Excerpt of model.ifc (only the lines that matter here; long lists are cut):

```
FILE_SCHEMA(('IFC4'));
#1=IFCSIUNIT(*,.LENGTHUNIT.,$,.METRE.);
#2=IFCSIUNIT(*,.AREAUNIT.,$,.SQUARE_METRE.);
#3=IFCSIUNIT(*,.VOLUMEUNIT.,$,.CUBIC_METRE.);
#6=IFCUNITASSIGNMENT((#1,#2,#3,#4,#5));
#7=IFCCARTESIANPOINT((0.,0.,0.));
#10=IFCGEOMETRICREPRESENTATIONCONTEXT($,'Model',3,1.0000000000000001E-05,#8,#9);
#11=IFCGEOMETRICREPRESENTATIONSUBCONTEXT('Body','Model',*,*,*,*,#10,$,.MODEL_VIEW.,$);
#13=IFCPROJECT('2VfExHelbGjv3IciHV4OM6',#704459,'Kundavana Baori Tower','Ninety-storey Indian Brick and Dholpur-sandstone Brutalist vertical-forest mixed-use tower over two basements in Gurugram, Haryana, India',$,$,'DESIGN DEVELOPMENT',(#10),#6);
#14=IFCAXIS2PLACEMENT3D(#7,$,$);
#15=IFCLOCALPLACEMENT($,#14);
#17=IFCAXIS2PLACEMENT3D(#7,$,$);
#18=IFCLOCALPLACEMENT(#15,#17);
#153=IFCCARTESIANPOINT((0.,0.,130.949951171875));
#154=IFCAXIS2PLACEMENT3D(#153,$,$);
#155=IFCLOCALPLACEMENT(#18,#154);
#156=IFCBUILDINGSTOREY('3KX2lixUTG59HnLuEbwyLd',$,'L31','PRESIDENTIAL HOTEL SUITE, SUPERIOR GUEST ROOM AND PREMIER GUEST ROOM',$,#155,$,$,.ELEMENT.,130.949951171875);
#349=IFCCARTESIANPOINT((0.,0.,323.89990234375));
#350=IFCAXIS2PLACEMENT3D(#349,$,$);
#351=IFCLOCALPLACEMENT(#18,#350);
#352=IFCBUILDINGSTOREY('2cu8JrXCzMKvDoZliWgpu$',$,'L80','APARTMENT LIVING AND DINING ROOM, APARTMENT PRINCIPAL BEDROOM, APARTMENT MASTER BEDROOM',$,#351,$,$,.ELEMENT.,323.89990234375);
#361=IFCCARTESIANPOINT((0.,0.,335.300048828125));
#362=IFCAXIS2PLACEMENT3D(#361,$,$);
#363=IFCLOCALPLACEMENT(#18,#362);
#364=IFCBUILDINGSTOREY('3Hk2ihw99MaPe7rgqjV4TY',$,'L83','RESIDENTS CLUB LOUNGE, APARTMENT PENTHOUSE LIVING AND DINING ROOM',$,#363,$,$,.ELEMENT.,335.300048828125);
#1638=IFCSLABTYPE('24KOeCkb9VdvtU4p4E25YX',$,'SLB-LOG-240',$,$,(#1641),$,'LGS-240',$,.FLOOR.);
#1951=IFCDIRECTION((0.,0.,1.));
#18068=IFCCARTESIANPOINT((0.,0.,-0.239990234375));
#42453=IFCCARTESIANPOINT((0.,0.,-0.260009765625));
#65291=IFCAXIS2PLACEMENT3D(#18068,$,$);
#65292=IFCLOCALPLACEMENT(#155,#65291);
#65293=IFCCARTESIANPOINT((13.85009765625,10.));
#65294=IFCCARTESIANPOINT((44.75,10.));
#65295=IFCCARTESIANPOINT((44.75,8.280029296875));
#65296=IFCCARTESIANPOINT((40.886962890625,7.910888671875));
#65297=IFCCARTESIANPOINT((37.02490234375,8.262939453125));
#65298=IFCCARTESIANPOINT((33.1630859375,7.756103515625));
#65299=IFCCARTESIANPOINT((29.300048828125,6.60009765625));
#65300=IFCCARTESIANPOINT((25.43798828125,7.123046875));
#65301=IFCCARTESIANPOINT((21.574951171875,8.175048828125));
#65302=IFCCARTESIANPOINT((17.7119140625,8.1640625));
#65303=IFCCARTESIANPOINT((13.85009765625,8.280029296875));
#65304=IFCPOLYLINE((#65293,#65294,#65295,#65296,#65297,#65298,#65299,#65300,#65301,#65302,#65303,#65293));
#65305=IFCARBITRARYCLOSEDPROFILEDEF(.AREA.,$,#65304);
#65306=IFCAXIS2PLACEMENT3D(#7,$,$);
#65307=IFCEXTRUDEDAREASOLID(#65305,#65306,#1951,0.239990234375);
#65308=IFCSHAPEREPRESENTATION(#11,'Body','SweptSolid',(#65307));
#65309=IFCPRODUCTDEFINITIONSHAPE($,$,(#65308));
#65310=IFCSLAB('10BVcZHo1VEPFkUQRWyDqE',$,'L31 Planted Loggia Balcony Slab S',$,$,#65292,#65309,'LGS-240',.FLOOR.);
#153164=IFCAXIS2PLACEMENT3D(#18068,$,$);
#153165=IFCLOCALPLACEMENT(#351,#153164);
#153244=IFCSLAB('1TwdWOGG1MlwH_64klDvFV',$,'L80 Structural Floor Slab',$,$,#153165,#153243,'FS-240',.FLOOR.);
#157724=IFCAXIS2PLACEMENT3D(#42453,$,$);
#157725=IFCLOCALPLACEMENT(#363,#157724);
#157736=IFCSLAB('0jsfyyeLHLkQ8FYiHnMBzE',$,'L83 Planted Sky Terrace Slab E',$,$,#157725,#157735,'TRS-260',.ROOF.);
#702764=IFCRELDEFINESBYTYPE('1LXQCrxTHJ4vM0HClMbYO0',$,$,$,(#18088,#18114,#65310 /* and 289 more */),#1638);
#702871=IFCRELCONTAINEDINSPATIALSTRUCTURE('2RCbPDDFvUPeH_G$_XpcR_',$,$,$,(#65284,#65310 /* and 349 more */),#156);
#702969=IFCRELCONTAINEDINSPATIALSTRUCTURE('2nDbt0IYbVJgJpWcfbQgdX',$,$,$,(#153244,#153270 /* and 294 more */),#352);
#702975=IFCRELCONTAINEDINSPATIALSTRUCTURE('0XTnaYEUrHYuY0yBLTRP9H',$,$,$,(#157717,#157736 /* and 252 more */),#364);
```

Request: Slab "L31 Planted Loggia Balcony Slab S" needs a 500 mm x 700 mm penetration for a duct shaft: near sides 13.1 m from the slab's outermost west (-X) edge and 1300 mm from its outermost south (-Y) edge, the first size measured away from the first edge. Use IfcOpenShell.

```python
import numpy as np
import ifcopenshell
import ifcopenshell.api.feature
import ifcopenshell.api.geometry
import ifcopenshell.api.root
import ifcopenshell.geom
import ifcopenshell.util.placement
import ifcopenshell.util.representation
import ifcopenshell.util.shape
import ifcopenshell.util.unit

model = ifcopenshell.open("model.ifc")
unit_scale = ifcopenshell.util.unit.calculate_unit_scale(model)
settings = ifcopenshell.geom.settings()


def volume(element):
    """Net volume in cubic metres, openings subtracted."""
    shape = ifcopenshell.geom.create_shape(settings, element)
    return ifcopenshell.util.shape.get_volume(shape.geometry)


slab = model.by_id(65310)
before = volume(slab)

# Extent in the slab's own axes, in metres. The edges named are its -X and -Y sides.
slab_shape = ifcopenshell.geom.create_shape(settings, slab)
vertices = ifcopenshell.util.shape.get_vertices(slab_shape.geometry)
x_min, y_min, bottom = vertices.min(axis=0)
top = vertices[:, 2].max()

opening = ifcopenshell.api.root.create_entity(model, ifc_class="IfcOpeningElement", name="Duct shaft opening", predefined_type="OPENING")
context = ifcopenshell.util.representation.get_context(model, "Model", "Body", "MODEL_VIEW")
width, depth = 0.5, 0.7
outline = [(0.0, 0.0), (width, 0.0), (width, depth), (0.0, depth), (0.0, 0.0)]
# Overshoot both faces by 50 mm so the cut is clean.
shape = ifcopenshell.api.geometry.add_slab_representation(
    model, context=context, depth=top - bottom + 0.1, polyline=outline
)
ifcopenshell.api.geometry.assign_representation(model, product=opening, representation=shape)

matrix = ifcopenshell.util.placement.get_local_placement(slab.ObjectPlacement)
matrix[:, 3] = matrix @ np.append(np.array([x_min + 13.1, y_min + 1.3, bottom - 0.05]) / unit_scale, 1.0)
ifcopenshell.api.geometry.edit_object_placement(model, product=opening, matrix=matrix, is_si=False)
ifcopenshell.api.feature.add_feature(model, feature=opening, element=slab)

after = volume(slab)

print(f"slab volume {before:.3f} -> {after:.3f} m3")

model.write("model-out.ifc")
```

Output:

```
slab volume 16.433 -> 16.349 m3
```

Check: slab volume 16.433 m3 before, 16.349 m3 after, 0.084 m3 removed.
